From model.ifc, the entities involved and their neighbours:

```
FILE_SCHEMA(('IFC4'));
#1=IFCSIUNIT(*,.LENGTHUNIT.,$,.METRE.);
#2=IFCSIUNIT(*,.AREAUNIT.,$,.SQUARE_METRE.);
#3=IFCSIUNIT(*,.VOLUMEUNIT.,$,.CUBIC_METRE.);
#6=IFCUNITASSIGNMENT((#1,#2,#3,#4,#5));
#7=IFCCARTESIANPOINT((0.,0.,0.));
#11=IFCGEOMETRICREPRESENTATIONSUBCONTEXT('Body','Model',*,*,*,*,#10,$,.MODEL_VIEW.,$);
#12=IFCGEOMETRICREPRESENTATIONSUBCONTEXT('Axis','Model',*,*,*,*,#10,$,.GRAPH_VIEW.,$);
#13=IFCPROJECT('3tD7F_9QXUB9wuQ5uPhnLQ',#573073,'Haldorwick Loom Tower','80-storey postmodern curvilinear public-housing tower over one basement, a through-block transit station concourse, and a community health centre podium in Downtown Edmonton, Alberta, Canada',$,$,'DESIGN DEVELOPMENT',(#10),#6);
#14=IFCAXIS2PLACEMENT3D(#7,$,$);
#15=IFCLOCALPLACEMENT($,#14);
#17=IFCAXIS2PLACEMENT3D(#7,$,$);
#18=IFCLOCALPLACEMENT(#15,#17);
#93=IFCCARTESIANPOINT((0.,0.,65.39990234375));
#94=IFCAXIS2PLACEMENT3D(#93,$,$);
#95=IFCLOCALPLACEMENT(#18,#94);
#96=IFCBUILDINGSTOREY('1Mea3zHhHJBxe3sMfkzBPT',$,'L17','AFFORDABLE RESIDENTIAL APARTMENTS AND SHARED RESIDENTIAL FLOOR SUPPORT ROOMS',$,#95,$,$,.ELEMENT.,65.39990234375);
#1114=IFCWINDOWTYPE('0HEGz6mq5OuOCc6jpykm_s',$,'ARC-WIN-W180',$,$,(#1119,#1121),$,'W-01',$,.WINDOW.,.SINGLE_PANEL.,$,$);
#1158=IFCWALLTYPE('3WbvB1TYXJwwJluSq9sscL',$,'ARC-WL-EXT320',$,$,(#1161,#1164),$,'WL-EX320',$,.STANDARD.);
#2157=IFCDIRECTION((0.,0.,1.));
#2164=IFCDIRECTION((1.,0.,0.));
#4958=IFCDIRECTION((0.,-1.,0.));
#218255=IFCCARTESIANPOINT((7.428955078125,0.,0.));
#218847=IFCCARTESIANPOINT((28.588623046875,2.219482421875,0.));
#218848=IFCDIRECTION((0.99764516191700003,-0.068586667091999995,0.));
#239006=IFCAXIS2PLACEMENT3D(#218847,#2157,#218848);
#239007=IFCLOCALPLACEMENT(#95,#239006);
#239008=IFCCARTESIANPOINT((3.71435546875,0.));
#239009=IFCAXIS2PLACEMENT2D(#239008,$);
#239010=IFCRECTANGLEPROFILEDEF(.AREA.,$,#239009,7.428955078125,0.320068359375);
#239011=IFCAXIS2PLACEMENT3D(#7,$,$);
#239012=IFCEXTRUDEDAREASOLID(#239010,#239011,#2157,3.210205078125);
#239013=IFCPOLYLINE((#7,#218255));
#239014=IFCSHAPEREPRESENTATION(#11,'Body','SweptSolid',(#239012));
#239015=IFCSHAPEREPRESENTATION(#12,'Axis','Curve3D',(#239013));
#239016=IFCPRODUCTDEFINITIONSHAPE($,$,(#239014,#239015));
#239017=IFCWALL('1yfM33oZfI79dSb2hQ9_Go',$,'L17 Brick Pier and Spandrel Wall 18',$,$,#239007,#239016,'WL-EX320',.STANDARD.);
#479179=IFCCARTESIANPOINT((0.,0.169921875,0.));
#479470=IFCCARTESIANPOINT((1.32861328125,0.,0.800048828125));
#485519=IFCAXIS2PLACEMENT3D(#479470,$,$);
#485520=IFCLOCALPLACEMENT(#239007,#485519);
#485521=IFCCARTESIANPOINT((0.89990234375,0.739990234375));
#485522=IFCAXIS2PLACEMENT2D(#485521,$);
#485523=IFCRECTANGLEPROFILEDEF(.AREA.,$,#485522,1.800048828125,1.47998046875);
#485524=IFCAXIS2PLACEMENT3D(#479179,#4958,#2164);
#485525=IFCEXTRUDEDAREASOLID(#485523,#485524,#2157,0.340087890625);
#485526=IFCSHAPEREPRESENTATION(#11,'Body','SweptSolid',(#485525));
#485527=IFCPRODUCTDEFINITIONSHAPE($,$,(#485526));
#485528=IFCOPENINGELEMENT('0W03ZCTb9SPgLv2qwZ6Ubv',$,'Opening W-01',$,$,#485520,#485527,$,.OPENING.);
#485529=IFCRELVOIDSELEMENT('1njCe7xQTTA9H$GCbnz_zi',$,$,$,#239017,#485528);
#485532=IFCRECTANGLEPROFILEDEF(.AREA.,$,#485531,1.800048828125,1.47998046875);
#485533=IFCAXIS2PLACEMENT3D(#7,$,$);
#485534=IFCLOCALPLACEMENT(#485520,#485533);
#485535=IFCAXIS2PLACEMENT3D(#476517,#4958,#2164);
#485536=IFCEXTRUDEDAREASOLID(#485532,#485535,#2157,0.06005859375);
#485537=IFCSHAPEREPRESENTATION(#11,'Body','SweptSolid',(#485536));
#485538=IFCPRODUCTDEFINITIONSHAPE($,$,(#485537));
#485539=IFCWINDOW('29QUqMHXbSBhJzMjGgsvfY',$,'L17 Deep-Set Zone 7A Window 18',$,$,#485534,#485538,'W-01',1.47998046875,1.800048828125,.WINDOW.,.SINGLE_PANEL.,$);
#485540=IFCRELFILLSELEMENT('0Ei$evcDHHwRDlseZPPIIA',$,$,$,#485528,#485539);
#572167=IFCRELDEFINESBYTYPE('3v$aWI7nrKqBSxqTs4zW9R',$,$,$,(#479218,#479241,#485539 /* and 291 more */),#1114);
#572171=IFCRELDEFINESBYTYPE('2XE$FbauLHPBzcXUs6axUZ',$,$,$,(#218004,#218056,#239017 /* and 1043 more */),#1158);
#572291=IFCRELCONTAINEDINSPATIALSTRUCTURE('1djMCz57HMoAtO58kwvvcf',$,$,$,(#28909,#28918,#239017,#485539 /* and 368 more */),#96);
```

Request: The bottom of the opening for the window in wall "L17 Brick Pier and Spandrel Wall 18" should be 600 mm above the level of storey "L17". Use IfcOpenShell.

```python
import numpy as np
import ifcopenshell
import ifcopenshell.api.geometry
import ifcopenshell.geom
import ifcopenshell.util.element
import ifcopenshell.util.placement
import ifcopenshell.util.shape
import ifcopenshell.util.unit

model = ifcopenshell.open("model.ifc")
unit_scale = ifcopenshell.util.unit.calculate_unit_scale(model)

window = model.by_guid("29QUqMHXbSBhJzMjGgsvfY")
opening = window.FillsVoids[0].RelatingOpeningElement
storey = ifcopenshell.util.element.get_container(window, ifc_class="IfcBuildingStorey")
level = ifcopenshell.util.placement.get_local_placement(storey.ObjectPlacement)[2, 3]

# The opening's origin need not be at the sill, so measure its lowest point.
shape = ifcopenshell.geom.create_shape(ifcopenshell.geom.settings(), opening)
bottom = ifcopenshell.util.shape.get_shape_bottom_elevation(shape, shape.geometry) / unit_scale
dz = level + 0.6 / unit_scale - bottom

shift = np.array([0.0, 0.0, dz])
# The window is placed relative to its opening, so it follows when the opening moves.
matrix = ifcopenshell.util.placement.get_local_placement(opening.ObjectPlacement)
matrix[:3, 3] += shift
ifcopenshell.api.geometry.edit_object_placement(
    model, product=opening, matrix=matrix, is_si=False, should_transform_children=True
)

print(f"moved by {dz * unit_scale:+.3f} m")

model.write("model_rev.ifc")
```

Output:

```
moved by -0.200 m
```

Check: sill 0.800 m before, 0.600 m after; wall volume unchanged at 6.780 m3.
